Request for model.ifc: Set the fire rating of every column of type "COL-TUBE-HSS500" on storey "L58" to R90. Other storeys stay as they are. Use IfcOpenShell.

First a look at what the model holds.

```python
import ifcopenshell
import ifcopenshell.util.element

model = ifcopenshell.open("model.ifc")
print(model.schema)
storey = next(s for s in model.by_type("IfcBuildingStorey") if s.Name == "L58")
columns = [e for e in ifcopenshell.util.element.get_decomposition(storey) if e.is_a("IfcColumn")]
seen = {}
for e in columns:
    element_type = ifcopenshell.util.element.get_type(e)
    key = (element_type.Name if element_type != e and element_type else None, ifcopenshell.util.element.get_pset(e, "Pset_ColumnCommon", "FireRating"))
    seen[key] = seen.get(key, 0) + 1
for (name, value), count in sorted(seen.items(), key=str):
    print(count, "x", name, "|", value)
```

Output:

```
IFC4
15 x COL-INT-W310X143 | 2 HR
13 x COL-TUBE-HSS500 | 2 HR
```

```python
import ifcopenshell
import ifcopenshell.api.pset
import ifcopenshell.util.element

model = ifcopenshell.open("model.ifc")

storey = next(s for s in model.by_type("IfcBuildingStorey") if s.Name == "L58")
columns = [e for e in ifcopenshell.util.element.get_decomposition(storey) if e.is_a("IfcColumn")]

count = 0
for e in columns:
    element_type = ifcopenshell.util.element.get_type(e)
    if element_type in (None, e) or element_type.Name != "COL-TUBE-HSS500":
        continue
    found = ifcopenshell.util.element.get_pset(e, "Pset_ColumnCommon", should_inherit=False)
    if found:
        pset = model.by_id(found["id"])
        if len(ifcopenshell.util.element.get_elements_by_pset(pset)) > 1:
            pset = ifcopenshell.api.pset.unshare_pset(model, products=[e], pset=pset)[0]
    else:
        pset = ifcopenshell.api.pset.add_pset(model, product=e, name="Pset_ColumnCommon")
    ifcopenshell.api.pset.edit_pset(model, pset=pset, properties={"FireRating": "R90"})
    count += 1

print(count, "columns updated")

model.write("model_updated.ifc")
```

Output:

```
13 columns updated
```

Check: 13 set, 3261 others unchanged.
